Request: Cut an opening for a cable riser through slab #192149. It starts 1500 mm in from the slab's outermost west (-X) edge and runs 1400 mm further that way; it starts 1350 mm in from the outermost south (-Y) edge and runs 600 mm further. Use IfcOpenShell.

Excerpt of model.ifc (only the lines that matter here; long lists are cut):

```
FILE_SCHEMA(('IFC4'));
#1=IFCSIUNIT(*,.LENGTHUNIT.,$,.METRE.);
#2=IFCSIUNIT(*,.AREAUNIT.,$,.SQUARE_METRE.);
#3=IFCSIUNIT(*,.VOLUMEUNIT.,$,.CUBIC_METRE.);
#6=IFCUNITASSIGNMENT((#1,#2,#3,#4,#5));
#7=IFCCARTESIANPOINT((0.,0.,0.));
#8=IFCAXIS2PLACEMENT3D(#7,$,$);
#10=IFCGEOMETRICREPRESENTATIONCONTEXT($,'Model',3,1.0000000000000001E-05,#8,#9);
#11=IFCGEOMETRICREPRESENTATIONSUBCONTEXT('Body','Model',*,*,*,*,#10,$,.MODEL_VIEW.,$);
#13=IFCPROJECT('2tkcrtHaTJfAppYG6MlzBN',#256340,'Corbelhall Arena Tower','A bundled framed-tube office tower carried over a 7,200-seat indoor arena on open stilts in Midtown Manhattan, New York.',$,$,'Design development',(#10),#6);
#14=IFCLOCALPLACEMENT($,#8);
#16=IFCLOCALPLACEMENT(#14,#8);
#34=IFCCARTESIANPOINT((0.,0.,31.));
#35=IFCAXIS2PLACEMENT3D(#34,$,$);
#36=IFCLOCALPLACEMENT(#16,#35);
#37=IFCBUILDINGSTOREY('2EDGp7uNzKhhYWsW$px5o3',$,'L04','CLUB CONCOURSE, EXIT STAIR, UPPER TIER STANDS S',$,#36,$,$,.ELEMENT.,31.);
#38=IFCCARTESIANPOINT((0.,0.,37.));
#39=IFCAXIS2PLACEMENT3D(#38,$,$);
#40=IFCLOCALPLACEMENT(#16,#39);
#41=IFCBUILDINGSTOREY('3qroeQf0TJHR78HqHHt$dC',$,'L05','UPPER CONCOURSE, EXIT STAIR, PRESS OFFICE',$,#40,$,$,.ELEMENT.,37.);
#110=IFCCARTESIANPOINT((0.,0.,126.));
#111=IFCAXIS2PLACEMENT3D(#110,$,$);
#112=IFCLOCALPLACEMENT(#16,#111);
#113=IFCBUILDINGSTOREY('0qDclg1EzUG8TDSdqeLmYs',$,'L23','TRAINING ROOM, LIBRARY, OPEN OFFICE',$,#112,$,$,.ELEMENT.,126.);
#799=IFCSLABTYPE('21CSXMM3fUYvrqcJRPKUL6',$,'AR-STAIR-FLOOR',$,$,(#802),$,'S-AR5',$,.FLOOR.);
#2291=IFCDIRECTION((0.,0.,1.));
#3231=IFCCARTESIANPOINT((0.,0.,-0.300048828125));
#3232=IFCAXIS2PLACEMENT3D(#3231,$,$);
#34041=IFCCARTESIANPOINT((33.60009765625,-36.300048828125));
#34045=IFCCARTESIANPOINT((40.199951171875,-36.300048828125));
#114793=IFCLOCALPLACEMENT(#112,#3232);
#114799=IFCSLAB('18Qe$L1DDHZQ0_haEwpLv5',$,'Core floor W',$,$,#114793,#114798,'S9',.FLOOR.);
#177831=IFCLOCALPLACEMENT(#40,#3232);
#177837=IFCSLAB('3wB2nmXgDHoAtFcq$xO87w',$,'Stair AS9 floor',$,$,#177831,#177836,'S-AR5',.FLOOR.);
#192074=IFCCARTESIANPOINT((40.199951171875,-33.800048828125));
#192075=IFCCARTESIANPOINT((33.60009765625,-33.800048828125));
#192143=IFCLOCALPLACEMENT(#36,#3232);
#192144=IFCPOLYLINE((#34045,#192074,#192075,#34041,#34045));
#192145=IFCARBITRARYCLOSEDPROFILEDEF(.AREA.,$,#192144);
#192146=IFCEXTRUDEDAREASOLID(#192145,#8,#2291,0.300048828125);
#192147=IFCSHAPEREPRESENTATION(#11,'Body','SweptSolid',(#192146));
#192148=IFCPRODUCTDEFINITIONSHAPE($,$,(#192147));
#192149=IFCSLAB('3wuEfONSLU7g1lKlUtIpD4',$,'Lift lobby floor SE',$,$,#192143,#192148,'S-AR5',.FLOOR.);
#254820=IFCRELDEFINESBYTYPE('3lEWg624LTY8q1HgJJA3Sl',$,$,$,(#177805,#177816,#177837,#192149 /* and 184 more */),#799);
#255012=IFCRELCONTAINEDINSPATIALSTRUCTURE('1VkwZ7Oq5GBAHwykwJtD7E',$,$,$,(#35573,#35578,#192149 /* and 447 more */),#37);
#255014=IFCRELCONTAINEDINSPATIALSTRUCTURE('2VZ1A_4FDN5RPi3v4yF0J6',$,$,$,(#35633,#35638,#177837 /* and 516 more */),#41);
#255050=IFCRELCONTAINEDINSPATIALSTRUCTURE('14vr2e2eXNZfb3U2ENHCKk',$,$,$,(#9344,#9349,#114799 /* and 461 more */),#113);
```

```python
import numpy as np
import ifcopenshell
import ifcopenshell.api.feature
import ifcopenshell.api.geometry
import ifcopenshell.api.root
import ifcopenshell.geom
import ifcopenshell.util.placement
import ifcopenshell.util.representation
import ifcopenshell.util.shape
import ifcopenshell.util.unit

model = ifcopenshell.open("model.ifc")
unit_scale = ifcopenshell.util.unit.calculate_unit_scale(model)
settings = ifcopenshell.geom.settings()


def volume(element):
    """Net volume in cubic metres, openings subtracted."""
    shape = ifcopenshell.geom.create_shape(settings, element)
    return ifcopenshell.util.shape.get_volume(shape.geometry)


slab = model.by_guid("3wuEfONSLU7g1lKlUtIpD4")
before = volume(slab)

# Extent in the slab's own axes, in metres. The edges named are its -X and -Y sides.
slab_shape = ifcopenshell.geom.create_shape(settings, slab)
vertices = ifcopenshell.util.shape.get_vertices(slab_shape.geometry)
x_min, y_min, bottom = vertices.min(axis=0)
top = vertices[:, 2].max()

opening = ifcopenshell.api.root.create_entity(model, ifc_class="IfcOpeningElement", name="Cable riser opening", predefined_type="OPENING")
context = ifcopenshell.util.representation.get_context(model, "Model", "Body", "MODEL_VIEW")
width, depth = 1.4, 0.6
outline = [(0.0, 0.0), (width, 0.0), (width, depth), (0.0, depth), (0.0, 0.0)]
# Overshoot both faces by 50 mm so the cut is clean.
shape = ifcopenshell.api.geometry.add_slab_representation(
    model, context=context, depth=top - bottom + 0.1, polyline=outline
)
ifcopenshell.api.geometry.assign_representation(model, product=opening, representation=shape)

matrix = ifcopenshell.util.placement.get_local_placement(slab.ObjectPlacement)
matrix[:, 3] = matrix @ np.append(np.array([x_min + 1.5, y_min + 1.35, bottom - 0.05]) / unit_scale, 1.0)
ifcopenshell.api.geometry.edit_object_placement(model, product=opening, matrix=matrix, is_si=False)
ifcopenshell.api.feature.add_feature(model, feature=opening, element=slab)

after = volume(slab)

print(f"slab volume {before:.3f} -> {after:.3f} m3")

model.write("model_updated.ifc")
```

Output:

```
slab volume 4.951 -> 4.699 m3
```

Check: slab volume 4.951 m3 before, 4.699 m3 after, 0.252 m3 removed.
